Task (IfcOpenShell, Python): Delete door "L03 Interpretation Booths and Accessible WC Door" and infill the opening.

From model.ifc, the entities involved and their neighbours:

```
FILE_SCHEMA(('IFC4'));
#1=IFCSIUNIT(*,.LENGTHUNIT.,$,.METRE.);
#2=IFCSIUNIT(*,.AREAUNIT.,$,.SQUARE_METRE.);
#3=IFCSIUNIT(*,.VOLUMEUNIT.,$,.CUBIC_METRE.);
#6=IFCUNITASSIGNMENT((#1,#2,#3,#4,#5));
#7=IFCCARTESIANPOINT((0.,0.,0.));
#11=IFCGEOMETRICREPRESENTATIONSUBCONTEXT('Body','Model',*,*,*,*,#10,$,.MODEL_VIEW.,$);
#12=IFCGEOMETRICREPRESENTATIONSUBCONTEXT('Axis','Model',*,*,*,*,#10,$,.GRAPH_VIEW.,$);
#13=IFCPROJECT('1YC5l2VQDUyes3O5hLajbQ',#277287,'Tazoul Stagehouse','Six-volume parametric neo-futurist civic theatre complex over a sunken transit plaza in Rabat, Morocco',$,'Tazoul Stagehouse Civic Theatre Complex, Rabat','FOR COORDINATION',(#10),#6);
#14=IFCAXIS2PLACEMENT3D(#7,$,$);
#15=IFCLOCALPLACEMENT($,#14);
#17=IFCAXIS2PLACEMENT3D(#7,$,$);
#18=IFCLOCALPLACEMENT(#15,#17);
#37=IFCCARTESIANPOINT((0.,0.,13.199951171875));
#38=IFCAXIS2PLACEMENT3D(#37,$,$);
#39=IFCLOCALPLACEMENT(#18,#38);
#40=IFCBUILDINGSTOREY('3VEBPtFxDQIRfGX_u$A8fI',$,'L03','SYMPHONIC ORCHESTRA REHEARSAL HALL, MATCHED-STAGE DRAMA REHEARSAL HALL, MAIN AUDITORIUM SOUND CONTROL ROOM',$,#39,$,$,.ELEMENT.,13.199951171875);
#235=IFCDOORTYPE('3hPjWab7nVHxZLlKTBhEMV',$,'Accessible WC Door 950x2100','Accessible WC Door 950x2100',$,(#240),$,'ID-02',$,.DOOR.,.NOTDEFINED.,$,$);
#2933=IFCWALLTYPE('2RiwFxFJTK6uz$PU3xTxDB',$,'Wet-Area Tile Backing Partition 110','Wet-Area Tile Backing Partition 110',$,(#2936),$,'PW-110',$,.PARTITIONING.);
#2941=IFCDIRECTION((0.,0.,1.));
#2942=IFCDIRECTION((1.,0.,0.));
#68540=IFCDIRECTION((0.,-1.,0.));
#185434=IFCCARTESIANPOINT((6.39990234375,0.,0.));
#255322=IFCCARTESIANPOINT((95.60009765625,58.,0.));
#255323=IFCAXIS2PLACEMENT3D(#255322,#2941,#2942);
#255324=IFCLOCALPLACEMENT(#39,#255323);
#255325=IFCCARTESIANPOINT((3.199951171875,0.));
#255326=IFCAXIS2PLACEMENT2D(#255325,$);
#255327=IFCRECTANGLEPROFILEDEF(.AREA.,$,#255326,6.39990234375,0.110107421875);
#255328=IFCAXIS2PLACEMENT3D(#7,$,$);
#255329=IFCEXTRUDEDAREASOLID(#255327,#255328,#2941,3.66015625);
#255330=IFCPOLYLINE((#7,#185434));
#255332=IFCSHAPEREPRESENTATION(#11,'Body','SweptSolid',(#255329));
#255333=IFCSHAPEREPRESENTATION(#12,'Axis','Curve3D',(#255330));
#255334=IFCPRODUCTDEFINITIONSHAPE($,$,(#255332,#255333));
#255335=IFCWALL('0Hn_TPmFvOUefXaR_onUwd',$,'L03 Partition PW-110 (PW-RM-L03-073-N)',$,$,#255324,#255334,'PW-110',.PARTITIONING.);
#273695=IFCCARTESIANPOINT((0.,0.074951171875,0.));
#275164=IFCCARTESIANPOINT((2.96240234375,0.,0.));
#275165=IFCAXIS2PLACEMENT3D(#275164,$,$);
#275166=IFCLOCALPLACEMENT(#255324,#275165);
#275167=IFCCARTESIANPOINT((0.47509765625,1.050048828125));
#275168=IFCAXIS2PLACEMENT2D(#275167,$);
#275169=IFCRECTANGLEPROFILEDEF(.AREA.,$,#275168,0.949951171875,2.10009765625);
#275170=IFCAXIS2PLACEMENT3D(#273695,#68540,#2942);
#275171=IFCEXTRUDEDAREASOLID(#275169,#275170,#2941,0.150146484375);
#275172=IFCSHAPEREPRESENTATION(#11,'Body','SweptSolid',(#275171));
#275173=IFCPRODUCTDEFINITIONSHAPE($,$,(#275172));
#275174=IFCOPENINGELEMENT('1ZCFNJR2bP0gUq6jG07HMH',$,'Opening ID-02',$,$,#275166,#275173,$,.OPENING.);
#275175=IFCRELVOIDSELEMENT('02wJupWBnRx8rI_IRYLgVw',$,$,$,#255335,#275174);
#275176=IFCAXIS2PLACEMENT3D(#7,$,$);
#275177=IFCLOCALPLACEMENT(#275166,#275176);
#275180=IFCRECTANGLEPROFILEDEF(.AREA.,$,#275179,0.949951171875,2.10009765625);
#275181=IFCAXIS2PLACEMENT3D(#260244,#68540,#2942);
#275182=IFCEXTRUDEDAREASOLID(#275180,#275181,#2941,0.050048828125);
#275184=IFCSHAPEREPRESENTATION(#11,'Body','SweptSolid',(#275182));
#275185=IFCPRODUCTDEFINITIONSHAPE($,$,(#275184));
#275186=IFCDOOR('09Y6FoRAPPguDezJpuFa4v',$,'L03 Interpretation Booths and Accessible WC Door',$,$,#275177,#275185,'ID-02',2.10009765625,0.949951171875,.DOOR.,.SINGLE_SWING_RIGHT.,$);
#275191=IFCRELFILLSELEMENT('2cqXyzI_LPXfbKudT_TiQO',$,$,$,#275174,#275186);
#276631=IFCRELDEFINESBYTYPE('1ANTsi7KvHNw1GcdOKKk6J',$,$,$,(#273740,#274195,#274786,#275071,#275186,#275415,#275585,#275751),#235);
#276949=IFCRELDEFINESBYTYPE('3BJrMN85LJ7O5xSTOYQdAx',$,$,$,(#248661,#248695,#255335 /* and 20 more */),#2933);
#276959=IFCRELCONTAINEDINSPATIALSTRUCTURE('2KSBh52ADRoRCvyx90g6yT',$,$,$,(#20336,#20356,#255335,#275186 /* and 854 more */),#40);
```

```python
import ifcopenshell
import ifcopenshell.api.feature
import ifcopenshell.api.root
import ifcopenshell.geom
import ifcopenshell.util.shape

model = ifcopenshell.open("model.ifc")
settings = ifcopenshell.geom.settings()


def volume(element):
    """Net volume in cubic metres, openings subtracted."""
    shape = ifcopenshell.geom.create_shape(settings, element)
    return ifcopenshell.util.shape.get_volume(shape.geometry)


door = model.by_guid("09Y6FoRAPPguDezJpuFa4v")
opening = door.FillsVoids[0].RelatingOpeningElement
wall = opening.VoidsElements[0].RelatingBuildingElement
before = volume(wall)

ifcopenshell.api.root.remove_product(model, product=door)
ifcopenshell.api.feature.remove_feature(model, feature=opening)

after = volume(wall)

print(f"wall volume {before:.3f} -> {after:.3f} m3")

model.write("model_v2.ifc")
```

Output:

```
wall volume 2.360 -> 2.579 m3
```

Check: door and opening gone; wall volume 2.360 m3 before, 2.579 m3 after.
